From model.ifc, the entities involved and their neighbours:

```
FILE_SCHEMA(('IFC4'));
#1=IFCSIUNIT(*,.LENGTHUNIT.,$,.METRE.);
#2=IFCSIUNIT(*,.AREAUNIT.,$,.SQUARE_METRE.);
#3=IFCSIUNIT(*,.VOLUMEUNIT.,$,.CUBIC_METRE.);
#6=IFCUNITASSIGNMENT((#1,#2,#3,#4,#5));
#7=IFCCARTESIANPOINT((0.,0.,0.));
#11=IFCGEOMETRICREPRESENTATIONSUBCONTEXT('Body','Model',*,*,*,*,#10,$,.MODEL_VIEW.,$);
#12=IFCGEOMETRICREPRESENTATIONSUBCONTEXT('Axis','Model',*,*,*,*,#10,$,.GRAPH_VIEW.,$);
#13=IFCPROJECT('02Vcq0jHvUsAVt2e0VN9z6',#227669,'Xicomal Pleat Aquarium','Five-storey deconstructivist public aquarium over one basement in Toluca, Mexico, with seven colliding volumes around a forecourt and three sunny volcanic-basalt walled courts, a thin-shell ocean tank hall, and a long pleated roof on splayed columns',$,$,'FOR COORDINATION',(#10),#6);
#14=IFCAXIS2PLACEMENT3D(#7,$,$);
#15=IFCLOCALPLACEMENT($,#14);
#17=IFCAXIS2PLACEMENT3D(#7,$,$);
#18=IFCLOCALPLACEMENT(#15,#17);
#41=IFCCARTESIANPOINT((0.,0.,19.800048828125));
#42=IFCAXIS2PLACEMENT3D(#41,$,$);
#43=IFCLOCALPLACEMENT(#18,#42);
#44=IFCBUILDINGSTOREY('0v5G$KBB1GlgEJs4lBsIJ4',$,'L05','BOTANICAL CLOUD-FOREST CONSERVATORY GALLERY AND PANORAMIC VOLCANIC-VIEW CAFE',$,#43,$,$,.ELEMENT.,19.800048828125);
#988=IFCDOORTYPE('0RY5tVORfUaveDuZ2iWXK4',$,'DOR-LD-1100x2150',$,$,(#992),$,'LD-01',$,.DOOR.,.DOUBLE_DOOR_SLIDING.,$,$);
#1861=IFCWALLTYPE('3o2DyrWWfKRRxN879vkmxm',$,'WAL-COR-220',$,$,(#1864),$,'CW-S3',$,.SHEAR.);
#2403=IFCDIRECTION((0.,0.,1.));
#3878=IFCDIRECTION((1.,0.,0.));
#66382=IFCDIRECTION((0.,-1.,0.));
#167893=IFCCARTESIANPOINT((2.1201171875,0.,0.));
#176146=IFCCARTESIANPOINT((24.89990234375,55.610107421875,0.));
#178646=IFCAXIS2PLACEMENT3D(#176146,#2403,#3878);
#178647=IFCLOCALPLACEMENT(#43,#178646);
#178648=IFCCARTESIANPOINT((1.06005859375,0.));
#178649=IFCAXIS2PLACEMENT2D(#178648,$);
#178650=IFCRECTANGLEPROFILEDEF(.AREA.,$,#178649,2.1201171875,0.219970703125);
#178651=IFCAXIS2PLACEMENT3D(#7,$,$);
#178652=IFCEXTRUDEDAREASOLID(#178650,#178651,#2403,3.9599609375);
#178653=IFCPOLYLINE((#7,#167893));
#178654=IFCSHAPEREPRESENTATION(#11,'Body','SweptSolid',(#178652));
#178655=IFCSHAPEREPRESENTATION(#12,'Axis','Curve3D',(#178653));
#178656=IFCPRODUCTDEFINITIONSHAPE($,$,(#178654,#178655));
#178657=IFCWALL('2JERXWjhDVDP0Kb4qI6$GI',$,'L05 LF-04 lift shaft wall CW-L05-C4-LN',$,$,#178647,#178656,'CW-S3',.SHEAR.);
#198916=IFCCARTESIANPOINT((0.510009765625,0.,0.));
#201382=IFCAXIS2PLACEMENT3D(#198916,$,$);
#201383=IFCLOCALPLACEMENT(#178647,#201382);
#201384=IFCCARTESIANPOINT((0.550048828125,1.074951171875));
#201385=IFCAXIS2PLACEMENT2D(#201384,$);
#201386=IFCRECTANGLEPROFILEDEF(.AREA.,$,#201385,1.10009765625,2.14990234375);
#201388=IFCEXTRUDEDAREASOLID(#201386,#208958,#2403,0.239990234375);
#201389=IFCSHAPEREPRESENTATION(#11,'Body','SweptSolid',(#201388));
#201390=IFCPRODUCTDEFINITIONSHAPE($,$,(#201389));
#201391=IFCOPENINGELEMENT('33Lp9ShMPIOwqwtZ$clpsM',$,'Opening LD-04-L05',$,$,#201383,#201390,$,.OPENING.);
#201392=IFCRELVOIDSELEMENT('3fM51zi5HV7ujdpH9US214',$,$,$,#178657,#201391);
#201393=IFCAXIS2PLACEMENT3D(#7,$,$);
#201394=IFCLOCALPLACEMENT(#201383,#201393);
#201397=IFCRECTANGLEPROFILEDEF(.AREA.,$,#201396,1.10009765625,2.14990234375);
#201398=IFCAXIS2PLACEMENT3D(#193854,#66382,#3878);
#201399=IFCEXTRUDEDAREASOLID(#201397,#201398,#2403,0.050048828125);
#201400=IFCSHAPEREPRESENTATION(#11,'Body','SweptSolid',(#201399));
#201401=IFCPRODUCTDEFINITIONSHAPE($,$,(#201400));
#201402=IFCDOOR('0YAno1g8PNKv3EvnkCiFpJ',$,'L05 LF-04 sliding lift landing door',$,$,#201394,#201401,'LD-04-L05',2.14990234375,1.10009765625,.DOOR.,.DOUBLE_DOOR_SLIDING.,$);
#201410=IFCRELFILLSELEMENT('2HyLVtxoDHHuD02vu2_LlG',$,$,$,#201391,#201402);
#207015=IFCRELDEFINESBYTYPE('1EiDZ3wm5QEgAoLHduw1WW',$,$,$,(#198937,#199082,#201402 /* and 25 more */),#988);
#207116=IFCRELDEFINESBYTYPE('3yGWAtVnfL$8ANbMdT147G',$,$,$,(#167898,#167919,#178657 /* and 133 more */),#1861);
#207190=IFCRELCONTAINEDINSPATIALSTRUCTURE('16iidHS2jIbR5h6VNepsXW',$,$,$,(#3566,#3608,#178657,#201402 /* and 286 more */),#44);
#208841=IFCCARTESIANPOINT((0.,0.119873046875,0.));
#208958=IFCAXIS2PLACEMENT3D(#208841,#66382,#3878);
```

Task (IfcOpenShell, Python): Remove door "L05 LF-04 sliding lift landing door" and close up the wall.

```python
import ifcopenshell
import ifcopenshell.api.feature
import ifcopenshell.api.root
import ifcopenshell.geom
import ifcopenshell.util.shape

model = ifcopenshell.open("model.ifc")
settings = ifcopenshell.geom.settings()


def volume(element):
    """Net volume in cubic metres, openings subtracted."""
    shape = ifcopenshell.geom.create_shape(settings, element)
    return ifcopenshell.util.shape.get_volume(shape.geometry)


door = model.by_id(201402)
opening = door.FillsVoids[0].RelatingOpeningElement
wall = opening.VoidsElements[0].RelatingBuildingElement
before = volume(wall)

ifcopenshell.api.root.remove_product(model, product=door)
ifcopenshell.api.feature.remove_feature(model, feature=opening)

after = volume(wall)

print(f"wall volume {before:.3f} -> {after:.3f} m3")

model.write("model-out.ifc")
```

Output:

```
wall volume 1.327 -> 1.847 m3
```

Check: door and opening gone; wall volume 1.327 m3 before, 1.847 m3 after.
